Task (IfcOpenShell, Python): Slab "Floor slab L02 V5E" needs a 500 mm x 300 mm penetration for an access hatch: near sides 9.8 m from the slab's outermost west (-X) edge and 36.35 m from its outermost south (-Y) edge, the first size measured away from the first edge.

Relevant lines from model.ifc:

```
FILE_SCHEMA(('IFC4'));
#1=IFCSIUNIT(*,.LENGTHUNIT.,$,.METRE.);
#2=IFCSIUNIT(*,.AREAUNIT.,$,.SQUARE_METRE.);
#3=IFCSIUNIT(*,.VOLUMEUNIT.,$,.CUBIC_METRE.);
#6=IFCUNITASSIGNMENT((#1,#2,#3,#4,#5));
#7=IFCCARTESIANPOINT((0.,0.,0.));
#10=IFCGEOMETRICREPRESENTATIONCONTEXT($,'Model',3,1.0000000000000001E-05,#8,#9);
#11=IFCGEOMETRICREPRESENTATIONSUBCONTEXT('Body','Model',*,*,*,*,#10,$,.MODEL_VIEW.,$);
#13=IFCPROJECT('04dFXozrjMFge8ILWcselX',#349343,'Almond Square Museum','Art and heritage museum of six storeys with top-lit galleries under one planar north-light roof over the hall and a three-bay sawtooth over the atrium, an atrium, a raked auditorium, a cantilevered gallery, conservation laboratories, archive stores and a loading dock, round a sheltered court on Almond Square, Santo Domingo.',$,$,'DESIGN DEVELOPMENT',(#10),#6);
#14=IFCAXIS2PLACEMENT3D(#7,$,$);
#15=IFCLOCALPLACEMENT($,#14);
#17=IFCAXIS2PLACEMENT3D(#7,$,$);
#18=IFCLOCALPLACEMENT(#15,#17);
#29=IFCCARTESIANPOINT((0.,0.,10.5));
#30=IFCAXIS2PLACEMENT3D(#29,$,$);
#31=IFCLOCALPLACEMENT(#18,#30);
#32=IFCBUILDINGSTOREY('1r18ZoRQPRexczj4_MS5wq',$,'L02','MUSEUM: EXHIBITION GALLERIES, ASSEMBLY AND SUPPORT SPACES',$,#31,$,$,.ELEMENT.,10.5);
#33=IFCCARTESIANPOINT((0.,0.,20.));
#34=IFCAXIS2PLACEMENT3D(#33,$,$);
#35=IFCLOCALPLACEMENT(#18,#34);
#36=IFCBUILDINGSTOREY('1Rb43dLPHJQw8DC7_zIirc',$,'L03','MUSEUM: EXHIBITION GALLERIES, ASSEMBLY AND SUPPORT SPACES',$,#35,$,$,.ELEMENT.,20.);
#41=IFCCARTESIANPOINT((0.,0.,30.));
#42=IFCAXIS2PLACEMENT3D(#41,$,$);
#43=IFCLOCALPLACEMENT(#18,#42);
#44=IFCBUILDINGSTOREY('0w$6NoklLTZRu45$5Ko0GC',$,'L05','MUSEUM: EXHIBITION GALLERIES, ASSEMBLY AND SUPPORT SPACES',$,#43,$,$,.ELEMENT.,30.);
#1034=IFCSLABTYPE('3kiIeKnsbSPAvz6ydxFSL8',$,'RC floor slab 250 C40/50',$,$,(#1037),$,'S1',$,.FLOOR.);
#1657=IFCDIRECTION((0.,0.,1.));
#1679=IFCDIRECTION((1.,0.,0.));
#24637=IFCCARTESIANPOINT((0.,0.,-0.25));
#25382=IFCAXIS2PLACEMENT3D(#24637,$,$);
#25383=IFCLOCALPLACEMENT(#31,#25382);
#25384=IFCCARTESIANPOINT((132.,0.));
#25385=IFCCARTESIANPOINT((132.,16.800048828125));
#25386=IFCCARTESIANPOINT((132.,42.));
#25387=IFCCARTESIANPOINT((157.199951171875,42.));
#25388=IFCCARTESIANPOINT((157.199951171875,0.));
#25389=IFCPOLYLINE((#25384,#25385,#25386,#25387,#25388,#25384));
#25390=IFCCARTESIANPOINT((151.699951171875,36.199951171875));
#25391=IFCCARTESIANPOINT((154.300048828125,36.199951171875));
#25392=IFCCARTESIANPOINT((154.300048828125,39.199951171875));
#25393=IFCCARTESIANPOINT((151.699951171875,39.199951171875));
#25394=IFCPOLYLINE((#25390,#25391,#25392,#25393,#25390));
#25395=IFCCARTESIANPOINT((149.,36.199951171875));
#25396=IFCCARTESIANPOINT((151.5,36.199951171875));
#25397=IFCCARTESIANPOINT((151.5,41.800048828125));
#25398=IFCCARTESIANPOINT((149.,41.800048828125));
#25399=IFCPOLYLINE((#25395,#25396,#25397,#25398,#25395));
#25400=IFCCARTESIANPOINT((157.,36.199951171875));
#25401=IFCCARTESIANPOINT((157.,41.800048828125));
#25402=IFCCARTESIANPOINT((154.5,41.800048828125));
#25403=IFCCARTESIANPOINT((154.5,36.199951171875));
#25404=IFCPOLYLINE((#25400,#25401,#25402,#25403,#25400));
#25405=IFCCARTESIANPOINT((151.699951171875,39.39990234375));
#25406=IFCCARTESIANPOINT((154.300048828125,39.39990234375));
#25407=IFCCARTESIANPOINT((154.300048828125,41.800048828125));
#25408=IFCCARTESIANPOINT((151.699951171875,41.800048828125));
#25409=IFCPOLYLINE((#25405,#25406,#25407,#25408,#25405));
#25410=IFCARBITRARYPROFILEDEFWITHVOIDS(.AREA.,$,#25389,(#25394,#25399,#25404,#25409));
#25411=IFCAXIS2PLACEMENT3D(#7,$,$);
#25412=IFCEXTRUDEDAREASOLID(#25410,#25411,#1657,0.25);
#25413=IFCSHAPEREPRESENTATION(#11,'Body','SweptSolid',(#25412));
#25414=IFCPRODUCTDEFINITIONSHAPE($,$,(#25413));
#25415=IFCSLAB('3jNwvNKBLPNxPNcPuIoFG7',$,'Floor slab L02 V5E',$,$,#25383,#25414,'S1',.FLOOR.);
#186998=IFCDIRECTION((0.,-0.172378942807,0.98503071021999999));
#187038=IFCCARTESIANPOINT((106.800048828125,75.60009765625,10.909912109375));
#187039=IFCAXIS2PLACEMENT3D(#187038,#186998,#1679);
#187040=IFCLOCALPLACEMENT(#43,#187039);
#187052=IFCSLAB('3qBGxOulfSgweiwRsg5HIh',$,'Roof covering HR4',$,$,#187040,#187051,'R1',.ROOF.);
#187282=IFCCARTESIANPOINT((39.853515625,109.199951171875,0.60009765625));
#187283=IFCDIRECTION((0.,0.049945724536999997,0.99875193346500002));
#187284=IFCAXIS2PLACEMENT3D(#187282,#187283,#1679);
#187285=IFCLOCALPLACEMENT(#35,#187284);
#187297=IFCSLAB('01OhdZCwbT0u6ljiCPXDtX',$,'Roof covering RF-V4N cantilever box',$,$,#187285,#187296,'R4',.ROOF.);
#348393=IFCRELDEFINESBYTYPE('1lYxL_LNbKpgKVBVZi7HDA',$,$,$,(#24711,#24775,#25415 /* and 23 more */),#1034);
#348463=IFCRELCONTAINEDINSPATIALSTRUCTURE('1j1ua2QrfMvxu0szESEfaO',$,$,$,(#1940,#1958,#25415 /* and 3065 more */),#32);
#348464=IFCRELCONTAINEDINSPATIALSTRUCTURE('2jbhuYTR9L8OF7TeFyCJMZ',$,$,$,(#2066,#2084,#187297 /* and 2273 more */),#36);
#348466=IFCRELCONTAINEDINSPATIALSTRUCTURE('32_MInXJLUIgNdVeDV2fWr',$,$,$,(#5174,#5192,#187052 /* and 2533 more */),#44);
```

```python
import numpy as np
import ifcopenshell
import ifcopenshell.api.feature
import ifcopenshell.api.geometry
import ifcopenshell.api.root
import ifcopenshell.geom
import ifcopenshell.util.placement
import ifcopenshell.util.representation
import ifcopenshell.util.shape
import ifcopenshell.util.unit

model = ifcopenshell.open("model.ifc")
unit_scale = ifcopenshell.util.unit.calculate_unit_scale(model)
settings = ifcopenshell.geom.settings()


def volume(element):
    """Net volume in cubic metres, openings subtracted."""
    shape = ifcopenshell.geom.create_shape(settings, element)
    return ifcopenshell.util.shape.get_volume(shape.geometry)


slab = model.by_guid("3jNwvNKBLPNxPNcPuIoFG7")
before = volume(slab)

# Extent in the slab's own axes, in metres. The edges named are its -X and -Y sides.
slab_shape = ifcopenshell.geom.create_shape(settings, slab)
vertices = ifcopenshell.util.shape.get_vertices(slab_shape.geometry)
x_min, y_min, bottom = vertices.min(axis=0)
top = vertices[:, 2].max()

opening = ifcopenshell.api.root.create_entity(model, ifc_class="IfcOpeningElement", name="Access hatch opening", predefined_type="OPENING")
context = ifcopenshell.util.representation.get_context(model, "Model", "Body", "MODEL_VIEW")
width, depth = 0.5, 0.3
outline = [(0.0, 0.0), (width, 0.0), (width, depth), (0.0, depth), (0.0, 0.0)]
# Overshoot both faces by 50 mm so the cut is clean.
shape = ifcopenshell.api.geometry.add_slab_representation(
    model, context=context, depth=top - bottom + 0.1, polyline=outline
)
ifcopenshell.api.geometry.assign_representation(model, product=opening, representation=shape)

matrix = ifcopenshell.util.placement.get_local_placement(slab.ObjectPlacement)
matrix[:, 3] = matrix @ np.append(np.array([x_min + 9.8, y_min + 36.35, bottom - 0.05]) / unit_scale, 1.0)
ifcopenshell.api.geometry.edit_object_placement(model, product=opening, matrix=matrix, is_si=False)
ifcopenshell.api.feature.add_feature(model, feature=opening, element=slab)

after = volume(slab)

print(f"slab volume {before:.3f} -> {after:.3f} m3")

model.write("model_updated.ifc")
```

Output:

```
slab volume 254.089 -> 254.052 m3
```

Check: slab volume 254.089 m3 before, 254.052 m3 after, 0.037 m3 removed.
